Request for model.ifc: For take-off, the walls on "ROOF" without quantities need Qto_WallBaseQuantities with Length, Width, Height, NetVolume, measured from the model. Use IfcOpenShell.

First a look at what the model holds.

```python
import ifcopenshell
import ifcopenshell.util.element
import ifcopenshell.util.unit

model = ifcopenshell.open("model.ifc")
print(model.schema)
for unit_type in ("LENGTHUNIT", "AREAUNIT", "VOLUMEUNIT"):
    print(unit_type, ifcopenshell.util.unit.calculate_unit_scale(model, unit_type))
storey = next(s for s in model.by_type("IfcBuildingStorey") if s.Name == "ROOF")
walls = [e for e in ifcopenshell.util.element.get_decomposition(storey) if e.is_a("IfcWall")]
for e in sorted(walls, key=lambda e: e.id()):
    print(e.id(), e.is_a(), e.Name, list(ifcopenshell.util.element.get_psets(e, qtos_only=True)), sep=" | ")
```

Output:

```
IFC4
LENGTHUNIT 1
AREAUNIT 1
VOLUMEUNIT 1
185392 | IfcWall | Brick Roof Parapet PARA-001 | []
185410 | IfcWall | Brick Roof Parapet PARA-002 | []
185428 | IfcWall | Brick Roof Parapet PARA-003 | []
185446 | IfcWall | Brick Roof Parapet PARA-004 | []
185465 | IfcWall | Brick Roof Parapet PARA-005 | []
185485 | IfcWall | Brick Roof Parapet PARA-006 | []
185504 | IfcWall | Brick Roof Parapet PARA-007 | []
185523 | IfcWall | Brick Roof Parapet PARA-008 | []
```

```python
import ifcopenshell
import ifcopenshell.api.pset
import ifcopenshell.geom
import ifcopenshell.util.element
import ifcopenshell.util.shape
import ifcopenshell.util.unit

model = ifcopenshell.open("model.ifc")
unit_scale = ifcopenshell.util.unit.calculate_unit_scale(model)
volume_scale = ifcopenshell.util.unit.calculate_unit_scale(model, "VOLUMEUNIT")
settings = ifcopenshell.geom.settings()

storey = next(s for s in model.by_type("IfcBuildingStorey") if s.Name == "ROOF")
walls = [e for e in ifcopenshell.util.element.get_decomposition(storey) if e.is_a("IfcWall")]

for e in sorted(walls, key=lambda e: e.id()):
    if ifcopenshell.util.element.get_psets(e, qtos_only=True, should_inherit=False):
        continue
    # Geometry comes back in metres, in the element's own axes.
    shape = ifcopenshell.geom.create_shape(settings, e)
    values = {
        "Length": ifcopenshell.util.shape.get_x(shape.geometry) / unit_scale,
        "Width": ifcopenshell.util.shape.get_y(shape.geometry) / unit_scale,
        "Height": ifcopenshell.util.shape.get_z(shape.geometry) / unit_scale,
        "NetVolume": ifcopenshell.util.shape.get_volume(shape.geometry) / volume_scale,
    }
    qto = ifcopenshell.api.pset.add_qto(model, product=e, name="Qto_WallBaseQuantities")
    ifcopenshell.api.pset.edit_qto(model, qto=qto, properties=values)
    print(e.id(), {k: round(v, 3) for k, v in values.items()})

model.write("model_v2.ifc")
```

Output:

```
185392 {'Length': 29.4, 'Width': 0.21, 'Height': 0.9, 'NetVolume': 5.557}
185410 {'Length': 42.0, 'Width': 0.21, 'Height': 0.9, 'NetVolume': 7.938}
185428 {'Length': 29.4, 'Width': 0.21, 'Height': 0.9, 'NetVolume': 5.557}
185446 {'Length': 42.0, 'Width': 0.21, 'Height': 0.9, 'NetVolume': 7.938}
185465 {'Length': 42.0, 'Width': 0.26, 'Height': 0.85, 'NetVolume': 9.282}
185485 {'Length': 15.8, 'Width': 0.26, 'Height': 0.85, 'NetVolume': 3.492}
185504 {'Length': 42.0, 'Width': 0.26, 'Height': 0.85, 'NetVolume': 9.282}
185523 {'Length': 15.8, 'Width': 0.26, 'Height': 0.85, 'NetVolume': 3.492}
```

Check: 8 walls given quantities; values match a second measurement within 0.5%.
